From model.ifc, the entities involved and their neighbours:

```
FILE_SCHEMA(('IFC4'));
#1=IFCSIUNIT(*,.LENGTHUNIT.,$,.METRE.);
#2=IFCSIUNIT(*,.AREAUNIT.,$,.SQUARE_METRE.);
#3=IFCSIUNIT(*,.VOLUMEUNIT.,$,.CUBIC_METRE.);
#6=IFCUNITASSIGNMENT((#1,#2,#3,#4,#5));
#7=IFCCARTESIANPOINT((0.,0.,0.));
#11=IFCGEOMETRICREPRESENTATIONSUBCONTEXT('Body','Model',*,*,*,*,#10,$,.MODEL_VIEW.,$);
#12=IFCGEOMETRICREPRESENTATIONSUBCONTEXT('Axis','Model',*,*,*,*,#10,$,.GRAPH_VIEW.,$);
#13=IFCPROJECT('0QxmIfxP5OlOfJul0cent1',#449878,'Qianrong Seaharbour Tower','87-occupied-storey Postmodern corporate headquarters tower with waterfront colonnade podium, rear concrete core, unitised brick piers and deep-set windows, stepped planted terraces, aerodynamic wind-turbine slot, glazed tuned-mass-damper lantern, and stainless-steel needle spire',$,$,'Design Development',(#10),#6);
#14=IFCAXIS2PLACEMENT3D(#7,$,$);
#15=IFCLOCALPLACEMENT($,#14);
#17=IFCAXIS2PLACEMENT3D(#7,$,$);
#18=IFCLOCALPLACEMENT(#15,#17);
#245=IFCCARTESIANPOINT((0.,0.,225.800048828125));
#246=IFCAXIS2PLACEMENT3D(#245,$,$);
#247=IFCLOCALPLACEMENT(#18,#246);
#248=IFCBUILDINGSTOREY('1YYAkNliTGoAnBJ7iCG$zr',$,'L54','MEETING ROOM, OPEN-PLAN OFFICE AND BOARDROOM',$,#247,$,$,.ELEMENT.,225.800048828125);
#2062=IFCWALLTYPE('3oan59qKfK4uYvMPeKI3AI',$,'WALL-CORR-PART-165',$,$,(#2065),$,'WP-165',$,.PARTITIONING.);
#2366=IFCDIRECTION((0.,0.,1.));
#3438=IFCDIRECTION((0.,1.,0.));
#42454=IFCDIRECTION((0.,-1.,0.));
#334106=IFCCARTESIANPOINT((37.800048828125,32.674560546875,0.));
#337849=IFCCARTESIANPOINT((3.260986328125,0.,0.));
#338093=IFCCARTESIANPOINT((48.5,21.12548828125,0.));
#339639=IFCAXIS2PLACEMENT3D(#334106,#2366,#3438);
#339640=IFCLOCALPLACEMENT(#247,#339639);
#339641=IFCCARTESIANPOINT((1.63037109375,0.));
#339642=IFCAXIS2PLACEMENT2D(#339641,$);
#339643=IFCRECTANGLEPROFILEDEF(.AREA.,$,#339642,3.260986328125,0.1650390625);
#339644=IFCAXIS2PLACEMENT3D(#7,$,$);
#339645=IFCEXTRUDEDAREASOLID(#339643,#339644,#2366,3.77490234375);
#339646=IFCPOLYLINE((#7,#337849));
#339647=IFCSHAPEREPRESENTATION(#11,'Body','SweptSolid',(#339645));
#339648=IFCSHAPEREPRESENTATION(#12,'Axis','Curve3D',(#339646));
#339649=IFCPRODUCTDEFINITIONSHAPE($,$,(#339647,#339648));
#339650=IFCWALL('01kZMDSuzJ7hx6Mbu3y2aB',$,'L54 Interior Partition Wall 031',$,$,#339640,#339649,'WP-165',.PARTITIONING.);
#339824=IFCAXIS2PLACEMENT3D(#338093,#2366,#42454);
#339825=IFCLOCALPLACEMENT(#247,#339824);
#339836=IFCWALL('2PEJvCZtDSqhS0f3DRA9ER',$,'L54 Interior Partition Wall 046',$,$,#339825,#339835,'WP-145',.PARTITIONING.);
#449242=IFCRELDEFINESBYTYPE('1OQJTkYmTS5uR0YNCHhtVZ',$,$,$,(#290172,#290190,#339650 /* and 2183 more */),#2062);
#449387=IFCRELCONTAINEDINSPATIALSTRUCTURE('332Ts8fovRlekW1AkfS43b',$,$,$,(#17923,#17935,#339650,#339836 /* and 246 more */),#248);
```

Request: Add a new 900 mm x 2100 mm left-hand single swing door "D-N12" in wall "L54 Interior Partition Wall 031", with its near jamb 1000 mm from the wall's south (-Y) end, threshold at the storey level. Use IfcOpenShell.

```python
import numpy as np
import ifcopenshell
import ifcopenshell.api.feature
import ifcopenshell.api.geometry
import ifcopenshell.api.root
import ifcopenshell.api.spatial
import ifcopenshell.geom
import ifcopenshell.util.element
import ifcopenshell.util.placement
import ifcopenshell.util.representation
import ifcopenshell.util.shape
import ifcopenshell.util.unit

model = ifcopenshell.open("model.ifc")
unit_scale = ifcopenshell.util.unit.calculate_unit_scale(model)
settings = ifcopenshell.geom.settings()


def volume(element):
    """Net volume in cubic metres, openings subtracted."""
    shape = ifcopenshell.geom.create_shape(settings, element)
    return ifcopenshell.util.shape.get_volume(shape.geometry)


wall = model.by_id(339650)
storey = ifcopenshell.util.element.get_container(wall, ifc_class="IfcBuildingStorey")
context = ifcopenshell.util.representation.get_context(model, "Model", "Body", "MODEL_VIEW")
before = volume(wall)

width, height, from_end, sill = 0.9, 2.1, 1, 0.0  # metres

# The wall runs along its own X axis, and the end named is its -X end.
wall_shape = ifcopenshell.geom.create_shape(settings, wall)
x, y, z = ifcopenshell.util.shape.get_vertices(wall_shape.geometry).T
start = x.min() + from_end
face, thickness = float(y.min()), float(y.max() - y.min())
wall_matrix = ifcopenshell.util.placement.get_local_placement(wall.ObjectPlacement)
level = ifcopenshell.util.placement.get_local_placement(storey.ObjectPlacement)[2, 3]


def in_wall(x, y):
    """Placement at x, y metres in the wall's axes, at sill height."""
    matrix = wall_matrix.copy()
    matrix[:, 3] = wall_matrix @ np.array([x / unit_scale, y / unit_scale, 0.0, 1.0])
    matrix[2, 3] = level + sill / unit_scale
    return matrix


# Opening: a box that overshoots both wall faces by 50 mm.
opening = ifcopenshell.api.root.create_entity(model, ifc_class="IfcOpeningElement", predefined_type="OPENING")
box = ifcopenshell.api.geometry.add_wall_representation(
    model, context=context, length=width, height=height, thickness=thickness + 0.1
)
ifcopenshell.api.geometry.assign_representation(model, product=opening, representation=box)
ifcopenshell.api.geometry.edit_object_placement(model, product=opening, matrix=in_wall(start, face - 0.05), is_si=False)
ifcopenshell.api.feature.add_feature(model, feature=opening, element=wall)

door = ifcopenshell.api.root.create_entity(model, ifc_class="IfcDoor", name="D-N12", predefined_type="DOOR")
door.OverallWidth, door.OverallHeight = width / unit_scale, height / unit_scale
door.OperationType = "SINGLE_SWING_LEFT"
body = ifcopenshell.api.geometry.add_door_representation(
    model,
    context=context,
    overall_width=door.OverallWidth,
    overall_height=door.OverallHeight,
    operation_type="SINGLE_SWING_LEFT",
    lining_properties={"LiningDepth": thickness / unit_scale, "ThresholdDepth": thickness / unit_scale},
)
ifcopenshell.api.geometry.assign_representation(model, product=door, representation=body)
ifcopenshell.api.spatial.assign_container(model, products=[door], relating_structure=storey)
ifcopenshell.api.feature.add_filling(model, opening=opening, element=door)

# The lining spans the wall, so the door starts at the wall face.
ifcopenshell.api.geometry.edit_object_placement(model, product=door, matrix=in_wall(start, face), is_si=False)

after = volume(wall)

print(f"wall volume {before:.3f} -> {after:.3f} m3")

model.write("model-out.ifc")
```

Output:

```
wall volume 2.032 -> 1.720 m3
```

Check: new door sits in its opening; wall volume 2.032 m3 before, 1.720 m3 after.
